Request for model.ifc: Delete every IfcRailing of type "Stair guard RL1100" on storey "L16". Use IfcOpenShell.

First a look at what the model holds.

```python
import ifcopenshell
import ifcopenshell.util.element

model = ifcopenshell.open("model.ifc")
print(model.schema)
storey = next(s for s in model.by_type("IfcBuildingStorey") if s.Name == "L16")
railings = [e for e in ifcopenshell.util.element.get_decomposition(storey) if e.is_a("IfcRailing")]
seen = {}
for e in railings:
    element_type = ifcopenshell.util.element.get_type(e)
    name = element_type.Name if element_type not in (None, e) else None
    seen[name] = seen.get(name, 0) + 1
for name, count in sorted(seen.items(), key=str):
    print(count, "x", name)
```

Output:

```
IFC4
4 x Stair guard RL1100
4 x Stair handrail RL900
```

```python
import ifcopenshell
import ifcopenshell.api.root
import ifcopenshell.util.element

model = ifcopenshell.open("model.ifc")

storey = next(s for s in model.by_type("IfcBuildingStorey") if s.Name == "L16")
railings = [e for e in ifcopenshell.util.element.get_decomposition(storey) if e.is_a("IfcRailing")]
targets = [e for e in railings if (t := ifcopenshell.util.element.get_type(e)) not in (None, e) and t.Name == "Stair guard RL1100"]

for e in targets:
    ifcopenshell.api.root.remove_product(model, product=e)
print(len(targets), "removed")

model.write("model_edited.ifc")
```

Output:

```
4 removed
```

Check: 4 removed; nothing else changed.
